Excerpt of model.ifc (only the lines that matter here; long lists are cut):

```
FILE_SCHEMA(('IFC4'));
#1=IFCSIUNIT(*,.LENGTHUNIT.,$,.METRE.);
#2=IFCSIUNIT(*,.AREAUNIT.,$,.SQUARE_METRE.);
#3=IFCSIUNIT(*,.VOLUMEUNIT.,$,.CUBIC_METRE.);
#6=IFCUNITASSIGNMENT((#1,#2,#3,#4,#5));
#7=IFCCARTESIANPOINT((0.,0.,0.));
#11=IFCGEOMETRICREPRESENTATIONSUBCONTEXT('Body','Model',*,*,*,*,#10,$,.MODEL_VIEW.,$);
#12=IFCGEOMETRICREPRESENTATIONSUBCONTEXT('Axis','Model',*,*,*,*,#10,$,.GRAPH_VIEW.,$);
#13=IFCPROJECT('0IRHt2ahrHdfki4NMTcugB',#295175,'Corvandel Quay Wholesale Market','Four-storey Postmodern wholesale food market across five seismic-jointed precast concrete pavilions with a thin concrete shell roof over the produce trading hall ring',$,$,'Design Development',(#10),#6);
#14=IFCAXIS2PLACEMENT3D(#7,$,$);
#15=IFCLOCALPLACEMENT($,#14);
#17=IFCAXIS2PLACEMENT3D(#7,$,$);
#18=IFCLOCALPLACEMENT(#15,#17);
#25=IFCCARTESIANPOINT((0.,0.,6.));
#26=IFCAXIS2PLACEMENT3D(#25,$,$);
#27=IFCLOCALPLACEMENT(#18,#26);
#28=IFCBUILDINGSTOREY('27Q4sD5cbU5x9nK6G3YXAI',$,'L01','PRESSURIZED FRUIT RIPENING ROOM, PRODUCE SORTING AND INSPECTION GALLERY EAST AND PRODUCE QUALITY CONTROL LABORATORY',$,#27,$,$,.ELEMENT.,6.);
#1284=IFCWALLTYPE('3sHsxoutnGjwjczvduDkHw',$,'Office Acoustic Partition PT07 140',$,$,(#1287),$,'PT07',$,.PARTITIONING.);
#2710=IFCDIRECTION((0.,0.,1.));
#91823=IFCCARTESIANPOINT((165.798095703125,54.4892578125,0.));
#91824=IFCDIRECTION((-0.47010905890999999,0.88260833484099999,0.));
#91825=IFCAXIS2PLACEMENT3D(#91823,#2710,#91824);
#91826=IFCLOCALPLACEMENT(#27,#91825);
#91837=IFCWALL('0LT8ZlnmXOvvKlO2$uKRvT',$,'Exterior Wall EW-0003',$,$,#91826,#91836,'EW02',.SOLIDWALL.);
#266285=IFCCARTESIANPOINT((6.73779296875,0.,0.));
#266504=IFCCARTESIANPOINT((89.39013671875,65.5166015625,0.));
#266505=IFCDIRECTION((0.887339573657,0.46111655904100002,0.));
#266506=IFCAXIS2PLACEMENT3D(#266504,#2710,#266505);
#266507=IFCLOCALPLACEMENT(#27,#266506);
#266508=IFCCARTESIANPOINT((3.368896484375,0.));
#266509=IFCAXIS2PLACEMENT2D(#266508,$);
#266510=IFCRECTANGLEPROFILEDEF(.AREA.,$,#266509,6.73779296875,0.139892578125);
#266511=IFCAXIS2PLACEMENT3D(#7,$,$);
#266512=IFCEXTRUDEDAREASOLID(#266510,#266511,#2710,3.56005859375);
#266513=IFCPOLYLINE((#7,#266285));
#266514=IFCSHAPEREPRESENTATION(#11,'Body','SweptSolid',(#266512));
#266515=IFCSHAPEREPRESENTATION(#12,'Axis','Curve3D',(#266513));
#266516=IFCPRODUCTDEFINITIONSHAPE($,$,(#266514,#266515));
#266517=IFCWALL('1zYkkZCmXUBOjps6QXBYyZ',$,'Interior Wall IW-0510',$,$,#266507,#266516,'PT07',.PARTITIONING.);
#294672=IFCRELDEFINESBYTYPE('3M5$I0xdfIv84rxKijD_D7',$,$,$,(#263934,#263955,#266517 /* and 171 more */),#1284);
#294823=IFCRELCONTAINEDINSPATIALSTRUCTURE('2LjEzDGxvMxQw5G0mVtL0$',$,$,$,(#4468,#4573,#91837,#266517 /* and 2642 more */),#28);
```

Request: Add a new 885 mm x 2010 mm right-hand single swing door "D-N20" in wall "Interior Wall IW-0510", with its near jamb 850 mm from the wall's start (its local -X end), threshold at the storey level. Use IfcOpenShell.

```python
import numpy as np
import ifcopenshell
import ifcopenshell.api.feature
import ifcopenshell.api.geometry
import ifcopenshell.api.root
import ifcopenshell.api.spatial
import ifcopenshell.geom
import ifcopenshell.util.element
import ifcopenshell.util.placement
import ifcopenshell.util.representation
import ifcopenshell.util.shape
import ifcopenshell.util.unit

model = ifcopenshell.open("model.ifc")
unit_scale = ifcopenshell.util.unit.calculate_unit_scale(model)
settings = ifcopenshell.geom.settings()


def volume(element):
    """Net volume in cubic metres, openings subtracted."""
    shape = ifcopenshell.geom.create_shape(settings, element)
    return ifcopenshell.util.shape.get_volume(shape.geometry)


wall = model.by_id(266517)
storey = ifcopenshell.util.element.get_container(wall, ifc_class="IfcBuildingStorey")
context = ifcopenshell.util.representation.get_context(model, "Model", "Body", "MODEL_VIEW")
before = volume(wall)

width, height, from_end, sill = 0.885, 2.01, 0.85, 0.0  # metres

# The wall runs along its own X axis, and the end named is its -X end.
wall_shape = ifcopenshell.geom.create_shape(settings, wall)
x, y, z = ifcopenshell.util.shape.get_vertices(wall_shape.geometry).T
start = x.min() + from_end
face, thickness = float(y.min()), float(y.max() - y.min())
wall_matrix = ifcopenshell.util.placement.get_local_placement(wall.ObjectPlacement)
level = ifcopenshell.util.placement.get_local_placement(storey.ObjectPlacement)[2, 3]


def in_wall(x, y):
    """Placement at x, y metres in the wall's axes, at sill height."""
    matrix = wall_matrix.copy()
    matrix[:, 3] = wall_matrix @ np.array([x / unit_scale, y / unit_scale, 0.0, 1.0])
    matrix[2, 3] = level + sill / unit_scale
    return matrix


# Opening: a box that overshoots both wall faces by 50 mm.
opening = ifcopenshell.api.root.create_entity(model, ifc_class="IfcOpeningElement", predefined_type="OPENING")
box = ifcopenshell.api.geometry.add_wall_representation(
    model, context=context, length=width, height=height, thickness=thickness + 0.1
)
ifcopenshell.api.geometry.assign_representation(model, product=opening, representation=box)
ifcopenshell.api.geometry.edit_object_placement(model, product=opening, matrix=in_wall(start, face - 0.05), is_si=False)
ifcopenshell.api.feature.add_feature(model, feature=opening, element=wall)

door = ifcopenshell.api.root.create_entity(model, ifc_class="IfcDoor", name="D-N20", predefined_type="DOOR")
door.OverallWidth, door.OverallHeight = width / unit_scale, height / unit_scale
door.OperationType = "SINGLE_SWING_RIGHT"
body = ifcopenshell.api.geometry.add_door_representation(
    model,
    context=context,
    overall_width=door.OverallWidth,
    overall_height=door.OverallHeight,
    operation_type="SINGLE_SWING_RIGHT",
    lining_properties={"LiningDepth": thickness / unit_scale, "ThresholdDepth": thickness / unit_scale},
)
ifcopenshell.api.geometry.assign_representation(model, product=door, representation=body)
ifcopenshell.api.spatial.assign_container(model, products=[door], relating_structure=storey)
ifcopenshell.api.feature.add_filling(model, opening=opening, element=door)

# The lining spans the wall, so the door starts at the wall face.
ifcopenshell.api.geometry.edit_object_placement(model, product=door, matrix=in_wall(start, face), is_si=False)

after = volume(wall)

print(f"wall volume {before:.3f} -> {after:.3f} m3")

model.write("model_updated.ifc")
```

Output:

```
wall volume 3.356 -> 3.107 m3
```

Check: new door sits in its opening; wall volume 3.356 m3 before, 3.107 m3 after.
